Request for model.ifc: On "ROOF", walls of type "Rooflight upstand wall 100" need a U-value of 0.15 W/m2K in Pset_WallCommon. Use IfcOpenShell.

First a look at what the model holds.

```python
import ifcopenshell
import ifcopenshell.util.element

model = ifcopenshell.open("model.ifc")
print(model.schema)
storey = next(s for s in model.by_type("IfcBuildingStorey") if s.Name == "ROOF")
walls = [e for e in ifcopenshell.util.element.get_decomposition(storey) if e.is_a("IfcWall")]
seen = {}
for e in walls:
    element_type = ifcopenshell.util.element.get_type(e)
    key = (element_type.Name if element_type != e and element_type else None, ifcopenshell.util.element.get_pset(e, "Pset_WallCommon", "ThermalTransmittance"))
    seen[key] = seen.get(key, 0) + 1
for (name, value), count in sorted(seen.items(), key=str):
    print(count, "x", name, "|", value)
```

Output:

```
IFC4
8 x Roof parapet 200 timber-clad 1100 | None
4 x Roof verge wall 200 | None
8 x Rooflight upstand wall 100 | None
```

```python
import ifcopenshell
import ifcopenshell.api.pset
import ifcopenshell.util.element

model = ifcopenshell.open("model.ifc")

storey = next(s for s in model.by_type("IfcBuildingStorey") if s.Name == "ROOF")
walls = [e for e in ifcopenshell.util.element.get_decomposition(storey) if e.is_a("IfcWall")]

count = 0
for e in walls:
    element_type = ifcopenshell.util.element.get_type(e)
    if element_type in (None, e) or element_type.Name != "Rooflight upstand wall 100":
        continue
    # add_pset returns the element's existing set when there is one.
    pset = ifcopenshell.api.pset.add_pset(model, product=e, name="Pset_WallCommon")
    ifcopenshell.api.pset.edit_pset(model, pset=pset, properties={"ThermalTransmittance": 0.15})
    count += 1

print(count, "walls updated")

model.write("model-out.ifc")
```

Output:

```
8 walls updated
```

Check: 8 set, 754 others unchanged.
